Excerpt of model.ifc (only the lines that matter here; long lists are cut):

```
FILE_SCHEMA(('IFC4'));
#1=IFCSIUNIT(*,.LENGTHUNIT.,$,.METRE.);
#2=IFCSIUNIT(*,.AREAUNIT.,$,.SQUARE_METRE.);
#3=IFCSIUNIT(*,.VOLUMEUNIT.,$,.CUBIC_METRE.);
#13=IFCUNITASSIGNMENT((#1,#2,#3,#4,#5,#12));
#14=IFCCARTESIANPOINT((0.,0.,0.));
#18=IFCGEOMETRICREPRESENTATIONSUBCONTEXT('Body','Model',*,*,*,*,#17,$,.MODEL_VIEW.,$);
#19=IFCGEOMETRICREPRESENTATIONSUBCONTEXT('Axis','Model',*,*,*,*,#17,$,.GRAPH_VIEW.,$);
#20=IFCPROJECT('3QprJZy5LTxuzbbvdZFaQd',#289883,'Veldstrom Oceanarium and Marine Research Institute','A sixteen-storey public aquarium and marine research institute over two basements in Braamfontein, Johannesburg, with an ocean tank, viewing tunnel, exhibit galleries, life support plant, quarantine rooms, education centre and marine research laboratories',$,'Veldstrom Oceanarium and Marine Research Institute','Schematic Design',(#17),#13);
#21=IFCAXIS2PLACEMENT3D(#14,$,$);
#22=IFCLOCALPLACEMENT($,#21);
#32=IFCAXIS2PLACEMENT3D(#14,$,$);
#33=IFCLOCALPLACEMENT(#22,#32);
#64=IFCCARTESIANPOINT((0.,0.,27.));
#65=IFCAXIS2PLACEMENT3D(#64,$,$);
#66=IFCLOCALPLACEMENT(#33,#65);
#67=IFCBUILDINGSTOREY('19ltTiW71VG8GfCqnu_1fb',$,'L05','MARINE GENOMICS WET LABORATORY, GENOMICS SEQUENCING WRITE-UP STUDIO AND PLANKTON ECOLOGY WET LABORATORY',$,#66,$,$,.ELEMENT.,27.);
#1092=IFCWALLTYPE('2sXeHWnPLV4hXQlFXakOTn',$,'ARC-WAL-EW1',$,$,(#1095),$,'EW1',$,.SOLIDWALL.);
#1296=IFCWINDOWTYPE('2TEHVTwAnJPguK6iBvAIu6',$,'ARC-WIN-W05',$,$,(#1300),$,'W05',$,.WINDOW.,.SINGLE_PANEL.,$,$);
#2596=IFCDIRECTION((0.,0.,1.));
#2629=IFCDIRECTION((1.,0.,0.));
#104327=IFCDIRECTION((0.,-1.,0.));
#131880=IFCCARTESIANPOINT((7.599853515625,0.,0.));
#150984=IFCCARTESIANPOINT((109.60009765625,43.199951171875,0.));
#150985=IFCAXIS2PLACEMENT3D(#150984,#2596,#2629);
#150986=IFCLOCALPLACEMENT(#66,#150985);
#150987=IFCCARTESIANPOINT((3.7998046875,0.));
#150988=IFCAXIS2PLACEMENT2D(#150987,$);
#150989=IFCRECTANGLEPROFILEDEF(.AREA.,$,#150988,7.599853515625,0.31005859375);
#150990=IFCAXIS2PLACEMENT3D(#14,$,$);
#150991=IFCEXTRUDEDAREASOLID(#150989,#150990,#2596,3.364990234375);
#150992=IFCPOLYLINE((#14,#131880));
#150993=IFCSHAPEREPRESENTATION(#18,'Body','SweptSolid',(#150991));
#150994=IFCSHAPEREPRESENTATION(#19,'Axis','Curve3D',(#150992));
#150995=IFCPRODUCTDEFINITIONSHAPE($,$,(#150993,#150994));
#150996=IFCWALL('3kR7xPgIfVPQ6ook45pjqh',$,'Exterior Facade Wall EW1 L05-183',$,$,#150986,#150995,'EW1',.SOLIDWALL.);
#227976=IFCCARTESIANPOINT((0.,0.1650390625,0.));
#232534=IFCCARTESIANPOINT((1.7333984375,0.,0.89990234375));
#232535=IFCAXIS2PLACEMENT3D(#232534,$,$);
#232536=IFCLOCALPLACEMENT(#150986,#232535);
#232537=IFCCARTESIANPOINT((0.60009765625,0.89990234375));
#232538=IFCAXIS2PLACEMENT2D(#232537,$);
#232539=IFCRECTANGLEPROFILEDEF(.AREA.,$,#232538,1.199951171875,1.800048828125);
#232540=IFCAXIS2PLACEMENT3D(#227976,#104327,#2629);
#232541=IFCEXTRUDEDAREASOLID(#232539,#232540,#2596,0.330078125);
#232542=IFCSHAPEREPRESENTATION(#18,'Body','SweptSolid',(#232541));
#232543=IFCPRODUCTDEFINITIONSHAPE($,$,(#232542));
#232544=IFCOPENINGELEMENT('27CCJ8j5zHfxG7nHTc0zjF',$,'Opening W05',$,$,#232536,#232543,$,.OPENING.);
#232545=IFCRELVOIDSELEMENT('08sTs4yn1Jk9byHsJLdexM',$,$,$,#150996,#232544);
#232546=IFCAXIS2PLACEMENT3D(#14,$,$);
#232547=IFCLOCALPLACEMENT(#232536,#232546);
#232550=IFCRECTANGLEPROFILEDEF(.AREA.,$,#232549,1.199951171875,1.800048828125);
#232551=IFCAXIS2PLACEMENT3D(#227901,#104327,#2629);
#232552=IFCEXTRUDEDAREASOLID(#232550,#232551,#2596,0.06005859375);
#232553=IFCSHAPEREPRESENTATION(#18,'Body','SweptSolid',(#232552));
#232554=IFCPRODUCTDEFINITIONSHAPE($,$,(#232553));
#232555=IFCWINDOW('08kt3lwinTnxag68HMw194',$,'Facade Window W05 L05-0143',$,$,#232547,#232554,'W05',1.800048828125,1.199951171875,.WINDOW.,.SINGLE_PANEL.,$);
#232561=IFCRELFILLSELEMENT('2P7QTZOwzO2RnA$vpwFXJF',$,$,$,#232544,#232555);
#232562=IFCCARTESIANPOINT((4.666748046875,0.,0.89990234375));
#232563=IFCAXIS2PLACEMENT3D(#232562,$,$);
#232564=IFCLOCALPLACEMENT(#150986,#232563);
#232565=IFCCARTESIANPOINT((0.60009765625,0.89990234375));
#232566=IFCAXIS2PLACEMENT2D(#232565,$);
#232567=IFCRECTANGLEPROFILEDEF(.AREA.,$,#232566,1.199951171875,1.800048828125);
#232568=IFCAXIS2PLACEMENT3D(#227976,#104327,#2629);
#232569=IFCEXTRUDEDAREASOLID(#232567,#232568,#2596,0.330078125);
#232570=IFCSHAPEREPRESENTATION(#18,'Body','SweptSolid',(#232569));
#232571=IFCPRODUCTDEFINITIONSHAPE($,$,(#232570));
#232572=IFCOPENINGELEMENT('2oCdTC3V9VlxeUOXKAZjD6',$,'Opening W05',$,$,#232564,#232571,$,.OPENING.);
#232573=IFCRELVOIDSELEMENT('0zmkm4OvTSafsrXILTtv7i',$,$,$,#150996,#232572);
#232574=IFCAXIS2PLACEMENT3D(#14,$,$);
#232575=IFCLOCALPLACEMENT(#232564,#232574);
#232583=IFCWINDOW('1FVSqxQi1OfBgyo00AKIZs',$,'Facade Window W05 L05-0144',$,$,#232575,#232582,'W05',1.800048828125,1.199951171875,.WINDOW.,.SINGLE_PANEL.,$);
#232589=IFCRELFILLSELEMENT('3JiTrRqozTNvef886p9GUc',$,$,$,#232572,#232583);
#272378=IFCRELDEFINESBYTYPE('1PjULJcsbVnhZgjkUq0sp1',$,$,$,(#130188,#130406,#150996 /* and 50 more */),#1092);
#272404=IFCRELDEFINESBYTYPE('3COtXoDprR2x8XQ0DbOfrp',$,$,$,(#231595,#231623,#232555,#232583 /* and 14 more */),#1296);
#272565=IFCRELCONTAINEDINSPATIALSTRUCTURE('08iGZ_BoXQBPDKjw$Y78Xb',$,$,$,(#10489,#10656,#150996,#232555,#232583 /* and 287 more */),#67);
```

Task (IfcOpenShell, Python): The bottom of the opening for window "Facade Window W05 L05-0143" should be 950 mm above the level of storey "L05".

```python
import numpy as np
import ifcopenshell
import ifcopenshell.api.geometry
import ifcopenshell.geom
import ifcopenshell.util.element
import ifcopenshell.util.placement
import ifcopenshell.util.shape
import ifcopenshell.util.unit

model = ifcopenshell.open("model.ifc")
unit_scale = ifcopenshell.util.unit.calculate_unit_scale(model)

window = model.by_id(232555)
opening = window.FillsVoids[0].RelatingOpeningElement
storey = ifcopenshell.util.element.get_container(window, ifc_class="IfcBuildingStorey")
level = ifcopenshell.util.placement.get_local_placement(storey.ObjectPlacement)[2, 3]

# The opening's origin need not be at the sill, so measure its lowest point.
shape = ifcopenshell.geom.create_shape(ifcopenshell.geom.settings(), opening)
bottom = ifcopenshell.util.shape.get_shape_bottom_elevation(shape, shape.geometry) / unit_scale
dz = level + 0.95 - bottom

shift = np.array([0.0, 0.0, dz])
# The window is placed relative to its opening, so it follows when the opening moves.
matrix = ifcopenshell.util.placement.get_local_placement(opening.ObjectPlacement)
matrix[:3, 3] += shift
ifcopenshell.api.geometry.edit_object_placement(
    model, product=opening, matrix=matrix, is_si=False, should_transform_children=True
)

print(f"moved by {dz * unit_scale:+.3f} m")

model.write("model_rev.ifc")
```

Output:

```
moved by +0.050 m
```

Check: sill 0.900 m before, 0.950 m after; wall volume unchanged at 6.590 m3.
